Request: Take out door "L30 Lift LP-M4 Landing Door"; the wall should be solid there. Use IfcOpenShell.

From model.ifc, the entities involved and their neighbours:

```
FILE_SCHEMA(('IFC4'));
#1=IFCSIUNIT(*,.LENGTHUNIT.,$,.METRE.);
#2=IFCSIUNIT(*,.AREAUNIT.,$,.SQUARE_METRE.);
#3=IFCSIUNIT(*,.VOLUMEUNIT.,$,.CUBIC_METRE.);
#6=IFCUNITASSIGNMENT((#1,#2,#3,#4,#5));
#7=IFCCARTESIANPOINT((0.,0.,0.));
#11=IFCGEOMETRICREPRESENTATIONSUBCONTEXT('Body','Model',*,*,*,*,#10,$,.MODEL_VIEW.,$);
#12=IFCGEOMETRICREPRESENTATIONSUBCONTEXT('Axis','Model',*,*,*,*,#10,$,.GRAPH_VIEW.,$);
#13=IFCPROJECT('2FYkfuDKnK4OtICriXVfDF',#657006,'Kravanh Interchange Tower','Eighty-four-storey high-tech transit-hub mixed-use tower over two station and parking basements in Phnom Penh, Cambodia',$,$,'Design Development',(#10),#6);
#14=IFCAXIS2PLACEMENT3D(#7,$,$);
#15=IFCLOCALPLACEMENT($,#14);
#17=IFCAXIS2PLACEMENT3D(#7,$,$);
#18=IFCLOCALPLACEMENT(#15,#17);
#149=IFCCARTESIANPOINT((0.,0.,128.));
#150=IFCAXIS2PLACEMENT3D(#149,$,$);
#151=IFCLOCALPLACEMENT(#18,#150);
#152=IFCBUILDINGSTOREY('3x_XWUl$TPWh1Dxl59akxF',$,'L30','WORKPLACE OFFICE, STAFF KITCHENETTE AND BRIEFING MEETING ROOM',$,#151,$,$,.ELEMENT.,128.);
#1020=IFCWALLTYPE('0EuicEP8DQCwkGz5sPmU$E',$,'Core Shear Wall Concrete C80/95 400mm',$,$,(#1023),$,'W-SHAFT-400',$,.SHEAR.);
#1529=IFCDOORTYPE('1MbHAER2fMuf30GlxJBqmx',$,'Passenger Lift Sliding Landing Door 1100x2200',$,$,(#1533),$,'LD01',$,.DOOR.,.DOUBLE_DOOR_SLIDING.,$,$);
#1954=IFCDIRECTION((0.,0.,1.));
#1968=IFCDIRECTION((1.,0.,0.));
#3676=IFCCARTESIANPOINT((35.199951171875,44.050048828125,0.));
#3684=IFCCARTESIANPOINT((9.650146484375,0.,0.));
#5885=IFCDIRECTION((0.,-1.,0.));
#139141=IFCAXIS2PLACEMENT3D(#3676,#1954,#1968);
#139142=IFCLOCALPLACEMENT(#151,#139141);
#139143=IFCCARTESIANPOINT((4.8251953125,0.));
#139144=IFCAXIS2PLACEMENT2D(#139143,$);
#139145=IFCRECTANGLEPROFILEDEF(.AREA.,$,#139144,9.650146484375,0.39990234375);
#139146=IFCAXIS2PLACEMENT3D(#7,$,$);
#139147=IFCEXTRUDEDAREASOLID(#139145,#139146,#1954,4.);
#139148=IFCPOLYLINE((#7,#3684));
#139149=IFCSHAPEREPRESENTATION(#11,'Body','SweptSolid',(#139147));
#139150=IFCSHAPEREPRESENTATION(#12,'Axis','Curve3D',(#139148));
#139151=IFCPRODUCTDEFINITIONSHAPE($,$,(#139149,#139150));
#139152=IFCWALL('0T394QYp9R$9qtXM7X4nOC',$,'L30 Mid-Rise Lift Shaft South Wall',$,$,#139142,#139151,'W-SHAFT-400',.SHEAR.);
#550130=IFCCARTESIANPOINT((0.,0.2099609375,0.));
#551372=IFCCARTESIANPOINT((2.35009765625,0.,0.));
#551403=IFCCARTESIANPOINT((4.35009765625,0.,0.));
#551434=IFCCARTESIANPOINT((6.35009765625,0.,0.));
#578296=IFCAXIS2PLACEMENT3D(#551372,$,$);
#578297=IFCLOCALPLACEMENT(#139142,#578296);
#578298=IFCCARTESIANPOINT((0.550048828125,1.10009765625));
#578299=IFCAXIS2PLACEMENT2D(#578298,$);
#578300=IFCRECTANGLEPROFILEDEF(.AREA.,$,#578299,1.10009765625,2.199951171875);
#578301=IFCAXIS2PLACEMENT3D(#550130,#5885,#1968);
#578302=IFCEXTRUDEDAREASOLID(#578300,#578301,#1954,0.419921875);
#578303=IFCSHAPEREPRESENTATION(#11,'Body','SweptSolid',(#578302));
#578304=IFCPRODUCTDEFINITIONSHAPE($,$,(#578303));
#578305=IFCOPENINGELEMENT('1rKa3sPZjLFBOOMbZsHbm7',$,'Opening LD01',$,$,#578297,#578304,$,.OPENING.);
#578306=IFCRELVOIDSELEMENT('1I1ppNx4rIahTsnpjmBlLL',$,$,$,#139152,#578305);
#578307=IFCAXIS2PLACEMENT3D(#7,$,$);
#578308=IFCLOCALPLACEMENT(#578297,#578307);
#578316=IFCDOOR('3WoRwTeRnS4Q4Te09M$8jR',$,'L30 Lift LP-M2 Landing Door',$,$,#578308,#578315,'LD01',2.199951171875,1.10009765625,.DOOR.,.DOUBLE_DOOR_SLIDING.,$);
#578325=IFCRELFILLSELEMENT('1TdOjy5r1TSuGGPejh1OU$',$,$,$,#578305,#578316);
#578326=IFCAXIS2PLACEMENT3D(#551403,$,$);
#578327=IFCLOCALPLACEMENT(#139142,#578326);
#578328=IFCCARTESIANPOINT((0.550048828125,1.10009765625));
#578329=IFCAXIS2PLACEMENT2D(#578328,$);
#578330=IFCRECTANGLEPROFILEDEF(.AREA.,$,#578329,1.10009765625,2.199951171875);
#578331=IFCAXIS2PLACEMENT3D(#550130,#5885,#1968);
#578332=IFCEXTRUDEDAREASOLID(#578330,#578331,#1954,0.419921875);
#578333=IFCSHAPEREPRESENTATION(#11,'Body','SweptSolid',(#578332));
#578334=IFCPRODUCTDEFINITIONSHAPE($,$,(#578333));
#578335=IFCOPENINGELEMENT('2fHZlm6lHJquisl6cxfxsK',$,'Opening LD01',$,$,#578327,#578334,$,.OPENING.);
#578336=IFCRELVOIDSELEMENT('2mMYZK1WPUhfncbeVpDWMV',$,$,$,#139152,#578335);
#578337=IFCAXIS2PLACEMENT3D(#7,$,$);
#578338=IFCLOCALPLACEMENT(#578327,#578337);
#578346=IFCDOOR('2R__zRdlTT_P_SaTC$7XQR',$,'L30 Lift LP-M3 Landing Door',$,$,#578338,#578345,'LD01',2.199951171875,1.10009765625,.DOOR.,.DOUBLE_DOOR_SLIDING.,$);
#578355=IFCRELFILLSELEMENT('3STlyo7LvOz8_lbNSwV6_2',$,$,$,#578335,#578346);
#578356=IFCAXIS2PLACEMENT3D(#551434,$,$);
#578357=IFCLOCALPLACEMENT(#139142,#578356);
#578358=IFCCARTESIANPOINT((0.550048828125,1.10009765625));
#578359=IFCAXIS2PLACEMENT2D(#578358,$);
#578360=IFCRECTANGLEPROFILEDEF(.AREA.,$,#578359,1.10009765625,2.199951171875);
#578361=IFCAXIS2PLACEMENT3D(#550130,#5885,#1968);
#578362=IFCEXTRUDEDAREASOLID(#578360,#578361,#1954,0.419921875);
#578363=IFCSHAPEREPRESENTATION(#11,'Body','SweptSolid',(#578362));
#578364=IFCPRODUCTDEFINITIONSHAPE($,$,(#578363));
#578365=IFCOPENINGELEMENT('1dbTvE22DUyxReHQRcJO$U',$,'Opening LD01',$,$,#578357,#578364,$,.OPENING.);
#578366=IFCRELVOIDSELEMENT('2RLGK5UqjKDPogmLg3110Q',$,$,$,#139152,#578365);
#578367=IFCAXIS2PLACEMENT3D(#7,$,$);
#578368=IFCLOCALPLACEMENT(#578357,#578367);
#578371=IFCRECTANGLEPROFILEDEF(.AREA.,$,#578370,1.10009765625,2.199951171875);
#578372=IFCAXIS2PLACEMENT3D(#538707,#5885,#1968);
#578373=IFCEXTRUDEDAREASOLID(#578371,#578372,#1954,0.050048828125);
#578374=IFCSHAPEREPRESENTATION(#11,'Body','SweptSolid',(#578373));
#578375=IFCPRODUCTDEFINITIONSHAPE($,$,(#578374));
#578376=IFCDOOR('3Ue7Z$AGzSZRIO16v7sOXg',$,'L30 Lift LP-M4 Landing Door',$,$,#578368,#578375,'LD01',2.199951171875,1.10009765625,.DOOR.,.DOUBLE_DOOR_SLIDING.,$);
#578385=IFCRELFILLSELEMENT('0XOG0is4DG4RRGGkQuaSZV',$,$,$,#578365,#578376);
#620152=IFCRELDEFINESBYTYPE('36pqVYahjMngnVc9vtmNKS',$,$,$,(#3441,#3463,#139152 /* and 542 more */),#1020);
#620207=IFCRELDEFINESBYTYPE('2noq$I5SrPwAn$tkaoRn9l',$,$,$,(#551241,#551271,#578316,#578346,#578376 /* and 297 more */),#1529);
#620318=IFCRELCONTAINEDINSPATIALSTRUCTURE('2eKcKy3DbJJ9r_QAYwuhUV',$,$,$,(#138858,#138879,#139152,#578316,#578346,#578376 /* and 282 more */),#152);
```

```python
import ifcopenshell
import ifcopenshell.api.feature
import ifcopenshell.api.root
import ifcopenshell.geom
import ifcopenshell.util.shape

model = ifcopenshell.open("model.ifc")
settings = ifcopenshell.geom.settings()


def volume(element):
    """Net volume in cubic metres, openings subtracted."""
    shape = ifcopenshell.geom.create_shape(settings, element)
    return ifcopenshell.util.shape.get_volume(shape.geometry)


door = model.by_guid("3Ue7Z$AGzSZRIO16v7sOXg")
opening = door.FillsVoids[0].RelatingOpeningElement
wall = opening.VoidsElements[0].RelatingBuildingElement
before = volume(wall)

ifcopenshell.api.root.remove_product(model, product=door)
ifcopenshell.api.feature.remove_feature(model, feature=opening)

after = volume(wall)

print(f"wall volume {before:.3f} -> {after:.3f} m3")

model.write("model_v2.ifc")
```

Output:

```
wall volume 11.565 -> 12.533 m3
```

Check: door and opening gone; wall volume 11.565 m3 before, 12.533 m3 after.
